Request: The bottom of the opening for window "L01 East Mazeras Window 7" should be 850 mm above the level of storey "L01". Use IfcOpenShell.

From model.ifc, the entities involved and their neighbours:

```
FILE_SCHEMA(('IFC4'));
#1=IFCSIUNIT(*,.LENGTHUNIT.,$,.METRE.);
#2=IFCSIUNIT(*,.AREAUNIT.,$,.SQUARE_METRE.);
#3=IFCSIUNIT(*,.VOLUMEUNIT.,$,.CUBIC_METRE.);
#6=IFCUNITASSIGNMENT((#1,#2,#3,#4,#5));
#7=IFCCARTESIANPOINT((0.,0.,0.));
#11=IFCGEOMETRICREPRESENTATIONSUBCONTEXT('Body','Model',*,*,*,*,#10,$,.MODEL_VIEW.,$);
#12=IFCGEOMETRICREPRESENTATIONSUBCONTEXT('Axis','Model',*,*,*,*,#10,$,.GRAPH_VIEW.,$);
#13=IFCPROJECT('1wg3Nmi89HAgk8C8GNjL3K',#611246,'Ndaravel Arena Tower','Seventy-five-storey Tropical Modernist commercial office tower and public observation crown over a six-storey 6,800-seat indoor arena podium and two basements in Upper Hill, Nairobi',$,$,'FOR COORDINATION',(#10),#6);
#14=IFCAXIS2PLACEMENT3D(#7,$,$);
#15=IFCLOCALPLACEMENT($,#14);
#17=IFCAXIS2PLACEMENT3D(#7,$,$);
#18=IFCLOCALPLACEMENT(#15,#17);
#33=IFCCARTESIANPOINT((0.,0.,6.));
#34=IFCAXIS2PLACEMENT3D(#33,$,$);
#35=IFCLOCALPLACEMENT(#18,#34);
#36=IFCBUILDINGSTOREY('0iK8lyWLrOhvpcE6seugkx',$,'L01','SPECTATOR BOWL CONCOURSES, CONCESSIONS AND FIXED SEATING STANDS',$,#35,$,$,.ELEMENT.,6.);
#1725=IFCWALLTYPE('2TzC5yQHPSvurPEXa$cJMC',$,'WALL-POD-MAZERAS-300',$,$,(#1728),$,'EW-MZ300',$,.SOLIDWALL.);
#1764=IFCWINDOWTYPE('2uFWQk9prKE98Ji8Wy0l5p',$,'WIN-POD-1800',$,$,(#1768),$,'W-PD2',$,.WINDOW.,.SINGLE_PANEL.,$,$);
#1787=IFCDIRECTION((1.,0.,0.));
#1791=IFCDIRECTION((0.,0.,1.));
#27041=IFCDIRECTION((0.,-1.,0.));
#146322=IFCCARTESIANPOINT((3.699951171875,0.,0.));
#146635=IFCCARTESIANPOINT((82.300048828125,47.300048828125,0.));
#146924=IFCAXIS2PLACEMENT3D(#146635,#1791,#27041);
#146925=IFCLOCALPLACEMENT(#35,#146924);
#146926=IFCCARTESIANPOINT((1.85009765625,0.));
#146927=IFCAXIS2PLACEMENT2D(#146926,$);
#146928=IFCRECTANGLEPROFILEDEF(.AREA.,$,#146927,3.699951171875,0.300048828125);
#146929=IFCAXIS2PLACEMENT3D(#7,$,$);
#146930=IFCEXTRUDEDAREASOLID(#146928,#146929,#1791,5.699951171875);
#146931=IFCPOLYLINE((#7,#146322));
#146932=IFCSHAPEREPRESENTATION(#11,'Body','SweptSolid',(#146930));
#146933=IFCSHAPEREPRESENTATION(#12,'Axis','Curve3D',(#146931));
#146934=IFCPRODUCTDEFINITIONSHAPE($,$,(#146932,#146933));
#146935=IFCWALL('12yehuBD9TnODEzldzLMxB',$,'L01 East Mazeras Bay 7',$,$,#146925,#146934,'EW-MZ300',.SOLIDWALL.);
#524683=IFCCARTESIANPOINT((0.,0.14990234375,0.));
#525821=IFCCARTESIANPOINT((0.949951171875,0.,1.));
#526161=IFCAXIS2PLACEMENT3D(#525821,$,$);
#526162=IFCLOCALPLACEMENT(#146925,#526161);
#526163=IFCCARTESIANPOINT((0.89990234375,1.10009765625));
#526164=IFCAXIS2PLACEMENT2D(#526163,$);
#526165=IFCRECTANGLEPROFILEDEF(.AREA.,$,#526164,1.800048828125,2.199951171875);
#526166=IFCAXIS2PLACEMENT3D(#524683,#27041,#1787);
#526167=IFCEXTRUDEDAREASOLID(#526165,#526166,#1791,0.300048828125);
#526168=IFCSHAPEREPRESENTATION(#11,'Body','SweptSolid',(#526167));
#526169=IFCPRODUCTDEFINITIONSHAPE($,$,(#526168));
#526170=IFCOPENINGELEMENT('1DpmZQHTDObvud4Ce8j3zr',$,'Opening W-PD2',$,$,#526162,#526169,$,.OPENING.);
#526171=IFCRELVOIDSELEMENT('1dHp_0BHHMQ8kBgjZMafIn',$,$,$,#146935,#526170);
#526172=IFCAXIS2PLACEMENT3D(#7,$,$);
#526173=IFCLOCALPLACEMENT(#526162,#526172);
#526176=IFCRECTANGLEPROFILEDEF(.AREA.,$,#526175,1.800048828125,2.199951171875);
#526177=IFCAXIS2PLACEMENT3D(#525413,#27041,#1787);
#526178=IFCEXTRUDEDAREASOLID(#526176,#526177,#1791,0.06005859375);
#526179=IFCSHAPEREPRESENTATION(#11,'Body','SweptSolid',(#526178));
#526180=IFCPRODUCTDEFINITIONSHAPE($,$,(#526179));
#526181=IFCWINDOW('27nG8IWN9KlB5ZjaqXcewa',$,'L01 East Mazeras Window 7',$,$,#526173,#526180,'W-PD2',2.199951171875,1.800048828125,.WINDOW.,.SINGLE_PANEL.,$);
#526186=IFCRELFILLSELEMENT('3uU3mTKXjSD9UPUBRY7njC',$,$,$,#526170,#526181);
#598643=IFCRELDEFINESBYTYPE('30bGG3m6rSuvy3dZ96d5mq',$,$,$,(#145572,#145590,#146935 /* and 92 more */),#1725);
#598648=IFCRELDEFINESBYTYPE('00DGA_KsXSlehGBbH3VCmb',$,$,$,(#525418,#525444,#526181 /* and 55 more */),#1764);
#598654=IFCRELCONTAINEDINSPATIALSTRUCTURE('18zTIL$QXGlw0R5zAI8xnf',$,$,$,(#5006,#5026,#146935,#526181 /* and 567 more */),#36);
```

```python
import numpy as np
import ifcopenshell
import ifcopenshell.api.geometry
import ifcopenshell.geom
import ifcopenshell.util.element
import ifcopenshell.util.placement
import ifcopenshell.util.shape
import ifcopenshell.util.unit

model = ifcopenshell.open("model.ifc")
unit_scale = ifcopenshell.util.unit.calculate_unit_scale(model)

window = model.by_guid("27nG8IWN9KlB5ZjaqXcewa")
opening = window.FillsVoids[0].RelatingOpeningElement
storey = ifcopenshell.util.element.get_container(window, ifc_class="IfcBuildingStorey")
level = ifcopenshell.util.placement.get_local_placement(storey.ObjectPlacement)[2, 3]

# The opening's origin need not be at the sill, so measure its lowest point.
shape = ifcopenshell.geom.create_shape(ifcopenshell.geom.settings(), opening)
bottom = ifcopenshell.util.shape.get_shape_bottom_elevation(shape, shape.geometry) / unit_scale
dz = level + 0.85 - bottom

shift = np.array([0.0, 0.0, dz])
# The window is placed relative to its opening, so it follows when the opening moves.
matrix = ifcopenshell.util.placement.get_local_placement(opening.ObjectPlacement)
matrix[:3, 3] += shift
ifcopenshell.api.geometry.edit_object_placement(
    model, product=opening, matrix=matrix, is_si=False, should_transform_children=True
)

print(f"moved by {dz * unit_scale:+.3f} m")

model.write("model_edited.ifc")
```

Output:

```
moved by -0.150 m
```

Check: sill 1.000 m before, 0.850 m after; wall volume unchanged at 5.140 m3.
